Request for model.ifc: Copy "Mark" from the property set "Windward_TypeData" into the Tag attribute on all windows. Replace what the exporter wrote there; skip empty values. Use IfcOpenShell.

First a look at what the model holds.

```python
import ifcopenshell
import ifcopenshell.util.element

model = ifcopenshell.open("model.ifc")
print(model.schema)
windows = model.by_type("IfcWindow")
print(len(windows), "windows")
for e in windows[:8]:
    source = ifcopenshell.util.element.get_pset(e, "Windward_TypeData", "Mark")
    target = e.Tag
    print(e.id(), repr(source), repr(target), sep=" | ")
```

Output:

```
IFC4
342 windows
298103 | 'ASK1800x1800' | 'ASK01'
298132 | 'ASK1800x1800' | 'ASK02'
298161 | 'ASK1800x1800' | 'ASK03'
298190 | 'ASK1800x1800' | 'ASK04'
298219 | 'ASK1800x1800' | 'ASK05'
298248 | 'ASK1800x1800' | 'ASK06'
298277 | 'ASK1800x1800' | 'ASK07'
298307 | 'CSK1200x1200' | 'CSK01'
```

```python
import ifcopenshell
import ifcopenshell.util.element

model = ifcopenshell.open("model.ifc")

count = 0
for e in model.by_type("IfcWindow"):
    value = ifcopenshell.util.element.get_pset(e, "Windward_TypeData", "Mark")
    current = e.Tag
    if not value or not value.strip() or current == value:
        continue
    e.Tag = value
    count += 1

print(count, "windows updated")

model.write("model_edited.ifc")
```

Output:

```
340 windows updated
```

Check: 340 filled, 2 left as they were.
